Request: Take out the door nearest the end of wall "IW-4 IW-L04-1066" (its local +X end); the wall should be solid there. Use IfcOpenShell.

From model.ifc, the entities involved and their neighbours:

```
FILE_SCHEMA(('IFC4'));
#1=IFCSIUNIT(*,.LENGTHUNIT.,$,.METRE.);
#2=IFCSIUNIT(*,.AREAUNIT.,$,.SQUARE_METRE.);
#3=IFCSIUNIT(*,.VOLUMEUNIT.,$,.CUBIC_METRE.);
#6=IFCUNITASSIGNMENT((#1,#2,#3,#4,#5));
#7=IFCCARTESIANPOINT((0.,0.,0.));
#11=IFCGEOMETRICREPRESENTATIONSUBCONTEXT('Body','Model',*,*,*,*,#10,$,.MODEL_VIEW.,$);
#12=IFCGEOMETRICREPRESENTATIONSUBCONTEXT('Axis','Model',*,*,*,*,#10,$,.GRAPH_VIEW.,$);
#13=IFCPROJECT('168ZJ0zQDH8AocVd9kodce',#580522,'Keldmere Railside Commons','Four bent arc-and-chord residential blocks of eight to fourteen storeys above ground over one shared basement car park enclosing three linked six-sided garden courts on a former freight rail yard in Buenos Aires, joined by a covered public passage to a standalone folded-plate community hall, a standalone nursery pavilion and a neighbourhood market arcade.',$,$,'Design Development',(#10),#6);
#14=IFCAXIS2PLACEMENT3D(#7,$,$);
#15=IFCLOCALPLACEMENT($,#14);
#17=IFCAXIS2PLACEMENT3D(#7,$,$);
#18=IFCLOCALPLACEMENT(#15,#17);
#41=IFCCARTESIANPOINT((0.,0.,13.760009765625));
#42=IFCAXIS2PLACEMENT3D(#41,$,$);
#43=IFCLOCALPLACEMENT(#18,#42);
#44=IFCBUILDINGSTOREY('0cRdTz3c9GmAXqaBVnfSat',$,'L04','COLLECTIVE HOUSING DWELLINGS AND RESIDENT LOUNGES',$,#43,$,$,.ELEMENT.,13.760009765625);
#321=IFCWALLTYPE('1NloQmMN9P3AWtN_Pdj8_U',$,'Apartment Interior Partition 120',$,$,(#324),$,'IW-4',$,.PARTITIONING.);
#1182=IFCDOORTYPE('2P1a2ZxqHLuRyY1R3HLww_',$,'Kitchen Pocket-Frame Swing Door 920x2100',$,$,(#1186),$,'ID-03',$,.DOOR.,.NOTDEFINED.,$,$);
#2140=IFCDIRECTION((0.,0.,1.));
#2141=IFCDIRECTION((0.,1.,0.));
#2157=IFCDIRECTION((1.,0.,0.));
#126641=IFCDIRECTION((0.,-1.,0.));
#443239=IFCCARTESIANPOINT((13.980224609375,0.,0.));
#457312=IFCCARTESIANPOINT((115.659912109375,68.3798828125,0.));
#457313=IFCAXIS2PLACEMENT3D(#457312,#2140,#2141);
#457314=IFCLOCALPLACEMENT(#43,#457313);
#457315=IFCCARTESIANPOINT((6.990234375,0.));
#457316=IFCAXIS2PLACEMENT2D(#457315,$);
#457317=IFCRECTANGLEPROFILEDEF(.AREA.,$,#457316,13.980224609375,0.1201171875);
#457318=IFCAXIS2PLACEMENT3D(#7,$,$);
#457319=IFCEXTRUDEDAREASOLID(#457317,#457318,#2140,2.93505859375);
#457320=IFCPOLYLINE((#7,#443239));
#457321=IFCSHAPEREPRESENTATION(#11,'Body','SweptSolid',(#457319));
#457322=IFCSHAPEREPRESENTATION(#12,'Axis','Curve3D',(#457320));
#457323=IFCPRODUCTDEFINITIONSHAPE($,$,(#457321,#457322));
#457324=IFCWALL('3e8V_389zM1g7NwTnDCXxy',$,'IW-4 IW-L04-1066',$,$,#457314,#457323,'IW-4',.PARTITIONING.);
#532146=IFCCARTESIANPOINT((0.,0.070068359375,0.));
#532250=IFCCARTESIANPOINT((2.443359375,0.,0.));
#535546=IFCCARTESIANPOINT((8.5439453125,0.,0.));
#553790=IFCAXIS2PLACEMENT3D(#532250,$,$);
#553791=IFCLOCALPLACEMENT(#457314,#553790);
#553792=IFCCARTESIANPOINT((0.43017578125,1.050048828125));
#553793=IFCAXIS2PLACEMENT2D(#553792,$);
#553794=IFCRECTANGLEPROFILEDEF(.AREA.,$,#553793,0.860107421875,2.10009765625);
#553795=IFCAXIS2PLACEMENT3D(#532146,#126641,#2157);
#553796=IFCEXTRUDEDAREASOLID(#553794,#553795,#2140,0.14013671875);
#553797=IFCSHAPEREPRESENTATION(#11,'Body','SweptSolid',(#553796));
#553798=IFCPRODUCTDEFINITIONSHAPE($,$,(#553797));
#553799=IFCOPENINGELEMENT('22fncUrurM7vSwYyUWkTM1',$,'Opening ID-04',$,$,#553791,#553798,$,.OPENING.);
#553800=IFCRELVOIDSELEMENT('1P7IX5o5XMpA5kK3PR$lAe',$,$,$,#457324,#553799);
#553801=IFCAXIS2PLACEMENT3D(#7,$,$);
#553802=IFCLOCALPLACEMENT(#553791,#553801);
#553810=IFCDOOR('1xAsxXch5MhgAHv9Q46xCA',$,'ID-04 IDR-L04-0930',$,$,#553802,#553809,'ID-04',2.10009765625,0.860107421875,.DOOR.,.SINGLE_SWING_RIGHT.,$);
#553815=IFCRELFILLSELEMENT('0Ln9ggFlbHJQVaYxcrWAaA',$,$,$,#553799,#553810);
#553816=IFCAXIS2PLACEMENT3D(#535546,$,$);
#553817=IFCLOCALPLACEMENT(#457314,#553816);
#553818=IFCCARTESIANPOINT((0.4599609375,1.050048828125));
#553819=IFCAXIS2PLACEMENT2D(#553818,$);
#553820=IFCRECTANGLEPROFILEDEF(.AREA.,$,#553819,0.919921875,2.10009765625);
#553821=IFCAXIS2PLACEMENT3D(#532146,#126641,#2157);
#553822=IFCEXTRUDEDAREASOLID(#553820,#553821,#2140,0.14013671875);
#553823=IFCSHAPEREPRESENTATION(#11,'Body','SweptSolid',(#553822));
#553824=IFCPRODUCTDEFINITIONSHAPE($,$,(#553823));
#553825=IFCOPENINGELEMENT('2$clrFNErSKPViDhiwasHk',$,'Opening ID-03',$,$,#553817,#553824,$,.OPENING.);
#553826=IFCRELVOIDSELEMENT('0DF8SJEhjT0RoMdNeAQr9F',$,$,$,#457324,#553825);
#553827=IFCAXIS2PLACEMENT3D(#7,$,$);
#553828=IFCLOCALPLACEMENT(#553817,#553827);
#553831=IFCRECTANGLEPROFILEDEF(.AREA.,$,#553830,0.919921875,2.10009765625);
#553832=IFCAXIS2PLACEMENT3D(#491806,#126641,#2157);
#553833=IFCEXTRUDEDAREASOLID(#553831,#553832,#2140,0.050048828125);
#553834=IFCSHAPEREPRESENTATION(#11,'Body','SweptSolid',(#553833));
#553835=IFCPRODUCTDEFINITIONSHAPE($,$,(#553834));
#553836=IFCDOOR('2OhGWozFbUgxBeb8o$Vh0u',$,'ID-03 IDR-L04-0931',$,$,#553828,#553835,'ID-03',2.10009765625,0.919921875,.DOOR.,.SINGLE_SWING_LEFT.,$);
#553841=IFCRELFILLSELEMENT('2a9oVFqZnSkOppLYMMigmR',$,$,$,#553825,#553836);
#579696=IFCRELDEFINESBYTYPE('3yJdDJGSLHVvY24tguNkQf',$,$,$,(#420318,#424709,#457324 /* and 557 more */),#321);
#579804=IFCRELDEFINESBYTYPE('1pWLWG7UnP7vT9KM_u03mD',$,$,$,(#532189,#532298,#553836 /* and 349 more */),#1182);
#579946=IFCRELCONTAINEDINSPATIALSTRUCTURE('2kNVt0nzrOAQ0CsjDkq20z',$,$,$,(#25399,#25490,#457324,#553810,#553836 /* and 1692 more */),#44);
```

```python
import ifcopenshell
import ifcopenshell.api.feature
import ifcopenshell.api.root
import ifcopenshell.geom
import ifcopenshell.util.shape

model = ifcopenshell.open("model.ifc")
settings = ifcopenshell.geom.settings()


def volume(element):
    """Net volume in cubic metres, openings subtracted."""
    shape = ifcopenshell.geom.create_shape(settings, element)
    return ifcopenshell.util.shape.get_volume(shape.geometry)


door = model.by_guid("2OhGWozFbUgxBeb8o$Vh0u")
opening = door.FillsVoids[0].RelatingOpeningElement
wall = opening.VoidsElements[0].RelatingBuildingElement
before = volume(wall)

ifcopenshell.api.root.remove_product(model, product=door)
ifcopenshell.api.feature.remove_feature(model, feature=opening)

after = volume(wall)

print(f"wall volume {before:.3f} -> {after:.3f} m3")

model.write("model_rev.ifc")
```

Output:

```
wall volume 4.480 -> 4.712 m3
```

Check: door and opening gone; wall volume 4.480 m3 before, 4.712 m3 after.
